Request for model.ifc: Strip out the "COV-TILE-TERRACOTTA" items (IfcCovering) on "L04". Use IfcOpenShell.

First a look at what the model holds.

```python
import ifcopenshell
import ifcopenshell.util.element

model = ifcopenshell.open("model.ifc")
print(model.schema)
storey = next(s for s in model.by_type("IfcBuildingStorey") if s.Name == "L04")
coverings = [e for e in ifcopenshell.util.element.get_decomposition(storey) if e.is_a("IfcCovering")]
seen = {}
for e in coverings:
    element_type = ifcopenshell.util.element.get_type(e)
    name = element_type.Name if element_type not in (None, e) else None
    seen[name] = seen.get(name, 0) + 1
for name, count in sorted(seen.items(), key=str):
    print(count, "x", name)
```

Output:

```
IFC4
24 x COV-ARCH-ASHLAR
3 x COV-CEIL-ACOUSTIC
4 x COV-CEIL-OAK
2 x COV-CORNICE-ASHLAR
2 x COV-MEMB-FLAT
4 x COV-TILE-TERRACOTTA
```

```python
import ifcopenshell
import ifcopenshell.api.root
import ifcopenshell.util.element

model = ifcopenshell.open("model.ifc")

storey = next(s for s in model.by_type("IfcBuildingStorey") if s.Name == "L04")
coverings = [e for e in ifcopenshell.util.element.get_decomposition(storey) if e.is_a("IfcCovering")]
targets = [e for e in coverings if (t := ifcopenshell.util.element.get_type(e)) not in (None, e) and t.Name == "COV-TILE-TERRACOTTA"]

for e in targets:
    ifcopenshell.api.root.remove_product(model, product=e)
print(len(targets), "removed")

model.write("model_updated.ifc")
```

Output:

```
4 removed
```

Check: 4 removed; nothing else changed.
